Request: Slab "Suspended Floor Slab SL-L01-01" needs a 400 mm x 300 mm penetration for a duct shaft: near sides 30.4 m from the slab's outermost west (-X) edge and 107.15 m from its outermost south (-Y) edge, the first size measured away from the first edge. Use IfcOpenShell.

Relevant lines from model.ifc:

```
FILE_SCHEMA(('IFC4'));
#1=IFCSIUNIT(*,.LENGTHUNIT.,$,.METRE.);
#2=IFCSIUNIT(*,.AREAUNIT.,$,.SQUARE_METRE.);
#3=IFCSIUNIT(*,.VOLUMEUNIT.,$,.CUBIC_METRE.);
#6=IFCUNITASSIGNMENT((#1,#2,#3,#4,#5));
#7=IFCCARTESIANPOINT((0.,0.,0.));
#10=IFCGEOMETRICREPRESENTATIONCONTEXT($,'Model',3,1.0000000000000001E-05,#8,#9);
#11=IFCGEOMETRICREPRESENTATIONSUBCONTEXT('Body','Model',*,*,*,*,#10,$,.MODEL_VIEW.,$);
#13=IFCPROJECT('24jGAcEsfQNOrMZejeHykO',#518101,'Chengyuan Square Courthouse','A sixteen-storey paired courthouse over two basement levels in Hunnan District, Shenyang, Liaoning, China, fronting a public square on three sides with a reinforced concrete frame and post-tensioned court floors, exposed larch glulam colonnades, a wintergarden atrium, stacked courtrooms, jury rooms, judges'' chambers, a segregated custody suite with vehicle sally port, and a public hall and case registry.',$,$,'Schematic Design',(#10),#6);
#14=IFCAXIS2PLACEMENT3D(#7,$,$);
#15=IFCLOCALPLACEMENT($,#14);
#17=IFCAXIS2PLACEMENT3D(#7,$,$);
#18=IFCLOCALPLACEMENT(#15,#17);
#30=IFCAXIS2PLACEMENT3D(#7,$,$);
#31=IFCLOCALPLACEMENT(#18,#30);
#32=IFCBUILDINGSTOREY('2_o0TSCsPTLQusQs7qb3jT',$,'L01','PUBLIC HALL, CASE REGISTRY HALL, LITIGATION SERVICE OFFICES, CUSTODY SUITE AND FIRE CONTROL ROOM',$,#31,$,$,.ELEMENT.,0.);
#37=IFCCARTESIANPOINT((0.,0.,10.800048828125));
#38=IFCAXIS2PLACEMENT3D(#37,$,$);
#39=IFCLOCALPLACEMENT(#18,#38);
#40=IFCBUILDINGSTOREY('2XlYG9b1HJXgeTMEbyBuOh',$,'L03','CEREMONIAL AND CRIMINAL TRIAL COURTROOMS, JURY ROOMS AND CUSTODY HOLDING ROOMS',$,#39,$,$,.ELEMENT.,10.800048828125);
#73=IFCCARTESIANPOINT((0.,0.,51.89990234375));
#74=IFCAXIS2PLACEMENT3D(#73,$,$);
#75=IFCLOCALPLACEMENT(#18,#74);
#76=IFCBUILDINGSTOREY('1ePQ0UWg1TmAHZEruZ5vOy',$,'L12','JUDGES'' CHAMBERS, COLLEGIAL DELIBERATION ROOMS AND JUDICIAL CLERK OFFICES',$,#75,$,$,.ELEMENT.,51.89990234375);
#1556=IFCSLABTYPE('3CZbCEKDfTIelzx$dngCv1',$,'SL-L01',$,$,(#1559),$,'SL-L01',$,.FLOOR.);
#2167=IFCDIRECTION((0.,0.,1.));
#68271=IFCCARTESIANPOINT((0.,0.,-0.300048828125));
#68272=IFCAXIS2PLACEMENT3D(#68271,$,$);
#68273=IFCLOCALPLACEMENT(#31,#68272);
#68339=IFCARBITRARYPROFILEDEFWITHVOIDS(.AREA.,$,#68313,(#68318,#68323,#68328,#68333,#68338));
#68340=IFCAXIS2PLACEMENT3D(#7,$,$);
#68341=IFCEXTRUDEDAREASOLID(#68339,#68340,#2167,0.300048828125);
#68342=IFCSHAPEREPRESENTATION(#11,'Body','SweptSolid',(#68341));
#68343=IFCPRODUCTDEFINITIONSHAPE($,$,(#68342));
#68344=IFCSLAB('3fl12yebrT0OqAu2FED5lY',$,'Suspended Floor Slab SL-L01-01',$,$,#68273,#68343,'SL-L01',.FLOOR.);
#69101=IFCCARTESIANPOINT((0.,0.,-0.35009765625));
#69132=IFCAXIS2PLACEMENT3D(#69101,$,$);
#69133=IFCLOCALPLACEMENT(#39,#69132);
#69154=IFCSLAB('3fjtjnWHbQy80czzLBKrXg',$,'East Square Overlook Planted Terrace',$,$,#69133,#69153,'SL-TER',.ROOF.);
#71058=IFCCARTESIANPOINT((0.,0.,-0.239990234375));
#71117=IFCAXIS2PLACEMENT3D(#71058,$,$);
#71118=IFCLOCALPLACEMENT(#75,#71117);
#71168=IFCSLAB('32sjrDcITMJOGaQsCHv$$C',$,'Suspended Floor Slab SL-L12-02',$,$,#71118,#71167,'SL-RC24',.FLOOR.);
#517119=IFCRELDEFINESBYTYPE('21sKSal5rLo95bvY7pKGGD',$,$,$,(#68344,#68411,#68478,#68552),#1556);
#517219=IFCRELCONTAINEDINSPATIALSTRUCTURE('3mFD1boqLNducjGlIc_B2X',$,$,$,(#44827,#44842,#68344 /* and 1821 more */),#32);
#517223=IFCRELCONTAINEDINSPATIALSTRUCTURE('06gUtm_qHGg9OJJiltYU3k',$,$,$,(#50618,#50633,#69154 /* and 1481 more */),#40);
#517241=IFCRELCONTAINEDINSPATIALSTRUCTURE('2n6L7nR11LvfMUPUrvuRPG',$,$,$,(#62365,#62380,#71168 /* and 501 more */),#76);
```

```python
import numpy as np
import ifcopenshell
import ifcopenshell.api.feature
import ifcopenshell.api.geometry
import ifcopenshell.api.root
import ifcopenshell.geom
import ifcopenshell.util.placement
import ifcopenshell.util.representation
import ifcopenshell.util.shape
import ifcopenshell.util.unit

model = ifcopenshell.open("model.ifc")
unit_scale = ifcopenshell.util.unit.calculate_unit_scale(model)
settings = ifcopenshell.geom.settings()


def volume(element):
    """Net volume in cubic metres, openings subtracted."""
    shape = ifcopenshell.geom.create_shape(settings, element)
    return ifcopenshell.util.shape.get_volume(shape.geometry)


slab = model.by_guid("3fl12yebrT0OqAu2FED5lY")
before = volume(slab)

# Extent in the slab's own axes, in metres. The edges named are its -X and -Y sides.
slab_shape = ifcopenshell.geom.create_shape(settings, slab)
vertices = ifcopenshell.util.shape.get_vertices(slab_shape.geometry)
x_min, y_min, bottom = vertices.min(axis=0)
top = vertices[:, 2].max()

opening = ifcopenshell.api.root.create_entity(model, ifc_class="IfcOpeningElement", name="Duct shaft opening", predefined_type="OPENING")
context = ifcopenshell.util.representation.get_context(model, "Model", "Body", "MODEL_VIEW")
width, depth = 0.4, 0.3
outline = [(0.0, 0.0), (width, 0.0), (width, depth), (0.0, depth), (0.0, 0.0)]
# Overshoot both faces by 50 mm so the cut is clean.
shape = ifcopenshell.api.geometry.add_slab_representation(
    model, context=context, depth=top - bottom + 0.1, polyline=outline
)
ifcopenshell.api.geometry.assign_representation(model, product=opening, representation=shape)

matrix = ifcopenshell.util.placement.get_local_placement(slab.ObjectPlacement)
matrix[:, 3] = matrix @ np.append(np.array([x_min + 30.4, y_min + 107.15, bottom - 0.05]) / unit_scale, 1.0)
ifcopenshell.api.geometry.edit_object_placement(model, product=opening, matrix=matrix, is_si=False)
ifcopenshell.api.feature.add_feature(model, feature=opening, element=slab)

after = volume(slab)

print(f"slab volume {before:.3f} -> {after:.3f} m3")

model.write("model_rev.ifc")
```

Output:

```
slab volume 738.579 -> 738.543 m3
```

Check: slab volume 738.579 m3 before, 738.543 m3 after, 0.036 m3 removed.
